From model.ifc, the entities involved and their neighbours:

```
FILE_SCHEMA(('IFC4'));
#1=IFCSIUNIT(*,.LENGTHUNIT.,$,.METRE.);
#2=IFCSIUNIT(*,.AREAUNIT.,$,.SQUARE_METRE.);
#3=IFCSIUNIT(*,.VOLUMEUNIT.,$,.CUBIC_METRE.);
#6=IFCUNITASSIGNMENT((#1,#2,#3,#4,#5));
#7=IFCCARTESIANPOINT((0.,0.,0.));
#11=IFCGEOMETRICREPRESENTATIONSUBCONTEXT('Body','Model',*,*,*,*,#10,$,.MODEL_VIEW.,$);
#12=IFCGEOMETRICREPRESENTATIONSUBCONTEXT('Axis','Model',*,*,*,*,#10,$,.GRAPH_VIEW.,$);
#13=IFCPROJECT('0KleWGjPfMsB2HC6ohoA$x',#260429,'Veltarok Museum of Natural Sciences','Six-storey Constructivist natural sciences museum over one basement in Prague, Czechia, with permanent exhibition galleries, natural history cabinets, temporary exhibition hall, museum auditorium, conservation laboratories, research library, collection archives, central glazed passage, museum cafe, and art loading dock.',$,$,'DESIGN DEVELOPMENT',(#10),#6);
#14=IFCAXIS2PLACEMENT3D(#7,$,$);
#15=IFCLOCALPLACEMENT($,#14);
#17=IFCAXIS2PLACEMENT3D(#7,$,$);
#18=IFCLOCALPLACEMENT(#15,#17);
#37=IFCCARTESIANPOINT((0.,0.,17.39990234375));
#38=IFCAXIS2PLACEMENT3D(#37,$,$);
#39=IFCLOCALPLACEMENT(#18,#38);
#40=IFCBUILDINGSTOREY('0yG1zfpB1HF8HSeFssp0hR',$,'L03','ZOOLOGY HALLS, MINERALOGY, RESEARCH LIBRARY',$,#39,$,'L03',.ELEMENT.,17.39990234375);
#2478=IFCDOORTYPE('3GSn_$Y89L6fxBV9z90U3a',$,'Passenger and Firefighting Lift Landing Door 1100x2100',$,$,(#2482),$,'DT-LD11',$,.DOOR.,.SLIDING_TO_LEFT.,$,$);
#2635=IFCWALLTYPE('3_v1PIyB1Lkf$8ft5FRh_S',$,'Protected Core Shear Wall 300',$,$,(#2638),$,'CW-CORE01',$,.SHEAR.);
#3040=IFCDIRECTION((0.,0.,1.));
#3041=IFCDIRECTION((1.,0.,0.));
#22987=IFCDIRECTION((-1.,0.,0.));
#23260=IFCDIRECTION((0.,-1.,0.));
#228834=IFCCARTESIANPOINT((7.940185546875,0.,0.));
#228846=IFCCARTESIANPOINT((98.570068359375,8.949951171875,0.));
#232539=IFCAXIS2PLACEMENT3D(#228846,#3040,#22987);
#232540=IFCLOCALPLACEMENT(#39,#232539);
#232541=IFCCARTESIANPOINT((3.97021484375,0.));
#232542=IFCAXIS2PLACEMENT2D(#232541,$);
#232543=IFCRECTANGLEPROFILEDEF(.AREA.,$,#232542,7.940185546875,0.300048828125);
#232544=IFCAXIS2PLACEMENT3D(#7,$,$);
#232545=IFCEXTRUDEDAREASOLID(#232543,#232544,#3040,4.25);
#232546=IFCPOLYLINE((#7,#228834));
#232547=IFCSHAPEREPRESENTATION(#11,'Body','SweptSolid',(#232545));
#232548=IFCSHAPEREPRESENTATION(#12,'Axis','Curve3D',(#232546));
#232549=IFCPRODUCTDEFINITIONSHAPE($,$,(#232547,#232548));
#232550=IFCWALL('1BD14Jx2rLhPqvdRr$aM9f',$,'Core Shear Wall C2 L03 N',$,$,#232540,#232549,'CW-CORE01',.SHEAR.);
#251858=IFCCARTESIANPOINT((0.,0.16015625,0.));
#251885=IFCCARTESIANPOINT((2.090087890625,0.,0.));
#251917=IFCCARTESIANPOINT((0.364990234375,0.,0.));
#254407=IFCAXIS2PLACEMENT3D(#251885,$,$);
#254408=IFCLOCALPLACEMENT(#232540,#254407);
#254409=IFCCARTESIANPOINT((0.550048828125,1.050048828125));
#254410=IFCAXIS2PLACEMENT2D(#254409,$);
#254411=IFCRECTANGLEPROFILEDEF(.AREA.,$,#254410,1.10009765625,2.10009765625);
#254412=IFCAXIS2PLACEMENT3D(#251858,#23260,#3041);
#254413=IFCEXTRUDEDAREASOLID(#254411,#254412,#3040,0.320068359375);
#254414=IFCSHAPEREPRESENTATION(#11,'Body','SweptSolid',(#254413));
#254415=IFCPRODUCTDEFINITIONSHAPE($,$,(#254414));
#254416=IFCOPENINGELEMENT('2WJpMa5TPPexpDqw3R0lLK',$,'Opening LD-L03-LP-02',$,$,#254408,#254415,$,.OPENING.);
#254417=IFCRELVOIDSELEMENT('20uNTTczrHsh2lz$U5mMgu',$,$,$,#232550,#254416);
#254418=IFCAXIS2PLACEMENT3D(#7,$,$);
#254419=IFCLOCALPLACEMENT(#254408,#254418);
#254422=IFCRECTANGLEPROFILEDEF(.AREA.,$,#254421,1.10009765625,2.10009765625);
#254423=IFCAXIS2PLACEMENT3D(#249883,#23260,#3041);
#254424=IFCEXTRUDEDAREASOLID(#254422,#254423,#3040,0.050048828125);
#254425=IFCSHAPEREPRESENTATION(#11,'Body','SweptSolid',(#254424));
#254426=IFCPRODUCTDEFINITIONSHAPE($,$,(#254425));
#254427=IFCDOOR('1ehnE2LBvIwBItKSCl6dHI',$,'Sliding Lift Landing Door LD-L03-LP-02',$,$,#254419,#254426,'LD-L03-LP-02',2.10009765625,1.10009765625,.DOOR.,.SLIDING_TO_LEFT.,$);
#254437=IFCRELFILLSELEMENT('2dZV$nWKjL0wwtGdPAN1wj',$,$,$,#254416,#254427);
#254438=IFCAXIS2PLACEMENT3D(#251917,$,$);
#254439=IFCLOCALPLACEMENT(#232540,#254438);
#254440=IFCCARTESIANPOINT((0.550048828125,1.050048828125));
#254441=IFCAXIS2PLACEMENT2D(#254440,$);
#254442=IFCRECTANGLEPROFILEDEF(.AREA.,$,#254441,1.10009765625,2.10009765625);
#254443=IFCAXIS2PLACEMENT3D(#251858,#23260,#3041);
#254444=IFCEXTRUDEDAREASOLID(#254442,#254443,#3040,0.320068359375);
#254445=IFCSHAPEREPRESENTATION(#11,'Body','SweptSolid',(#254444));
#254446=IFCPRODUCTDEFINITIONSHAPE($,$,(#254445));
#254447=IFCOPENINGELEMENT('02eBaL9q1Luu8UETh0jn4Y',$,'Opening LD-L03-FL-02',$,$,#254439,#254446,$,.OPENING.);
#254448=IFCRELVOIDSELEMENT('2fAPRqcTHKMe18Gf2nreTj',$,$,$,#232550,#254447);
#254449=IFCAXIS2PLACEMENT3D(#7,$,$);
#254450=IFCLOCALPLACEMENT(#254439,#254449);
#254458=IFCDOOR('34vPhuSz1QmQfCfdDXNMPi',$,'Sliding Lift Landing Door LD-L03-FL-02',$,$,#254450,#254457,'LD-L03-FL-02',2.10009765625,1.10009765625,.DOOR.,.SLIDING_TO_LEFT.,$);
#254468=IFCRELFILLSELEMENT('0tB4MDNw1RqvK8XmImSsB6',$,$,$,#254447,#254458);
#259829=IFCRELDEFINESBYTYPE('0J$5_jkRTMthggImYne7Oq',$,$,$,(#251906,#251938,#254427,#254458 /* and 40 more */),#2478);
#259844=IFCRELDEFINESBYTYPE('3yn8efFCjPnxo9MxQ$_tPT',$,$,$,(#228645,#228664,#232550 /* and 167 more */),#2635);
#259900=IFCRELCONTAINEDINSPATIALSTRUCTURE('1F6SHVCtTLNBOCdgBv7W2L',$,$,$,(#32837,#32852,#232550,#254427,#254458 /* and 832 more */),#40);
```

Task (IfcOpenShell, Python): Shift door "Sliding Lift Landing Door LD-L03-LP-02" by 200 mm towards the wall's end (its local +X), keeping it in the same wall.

```python
import ifcopenshell
import ifcopenshell.api.geometry
import ifcopenshell.util.placement
import ifcopenshell.util.unit

model = ifcopenshell.open("model.ifc")
unit_scale = ifcopenshell.util.unit.calculate_unit_scale(model)

door = model.by_guid("1ehnE2LBvIwBItKSCl6dHI")
opening = door.FillsVoids[0].RelatingOpeningElement
wall = opening.VoidsElements[0].RelatingBuildingElement

wall_matrix = ifcopenshell.util.placement.get_local_placement(wall.ObjectPlacement)
shift = wall_matrix[:3, 0] * 0.2 / unit_scale
before = ifcopenshell.util.placement.get_local_placement(door.ObjectPlacement)[:3, 3].copy()

# The door is placed relative to its opening, so it follows when the opening moves.
matrix = ifcopenshell.util.placement.get_local_placement(opening.ObjectPlacement)
matrix[:3, 3] += shift
ifcopenshell.api.geometry.edit_object_placement(
    model, product=opening, matrix=matrix, is_si=False, should_transform_children=True
)

after = ifcopenshell.util.placement.get_local_placement(door.ObjectPlacement)[:3, 3]
print("door moved by", (after - before).round(3) + 0.0)

model.write("model_updated.ifc")
```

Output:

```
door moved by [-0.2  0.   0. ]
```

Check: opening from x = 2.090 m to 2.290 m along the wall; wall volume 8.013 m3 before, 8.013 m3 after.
